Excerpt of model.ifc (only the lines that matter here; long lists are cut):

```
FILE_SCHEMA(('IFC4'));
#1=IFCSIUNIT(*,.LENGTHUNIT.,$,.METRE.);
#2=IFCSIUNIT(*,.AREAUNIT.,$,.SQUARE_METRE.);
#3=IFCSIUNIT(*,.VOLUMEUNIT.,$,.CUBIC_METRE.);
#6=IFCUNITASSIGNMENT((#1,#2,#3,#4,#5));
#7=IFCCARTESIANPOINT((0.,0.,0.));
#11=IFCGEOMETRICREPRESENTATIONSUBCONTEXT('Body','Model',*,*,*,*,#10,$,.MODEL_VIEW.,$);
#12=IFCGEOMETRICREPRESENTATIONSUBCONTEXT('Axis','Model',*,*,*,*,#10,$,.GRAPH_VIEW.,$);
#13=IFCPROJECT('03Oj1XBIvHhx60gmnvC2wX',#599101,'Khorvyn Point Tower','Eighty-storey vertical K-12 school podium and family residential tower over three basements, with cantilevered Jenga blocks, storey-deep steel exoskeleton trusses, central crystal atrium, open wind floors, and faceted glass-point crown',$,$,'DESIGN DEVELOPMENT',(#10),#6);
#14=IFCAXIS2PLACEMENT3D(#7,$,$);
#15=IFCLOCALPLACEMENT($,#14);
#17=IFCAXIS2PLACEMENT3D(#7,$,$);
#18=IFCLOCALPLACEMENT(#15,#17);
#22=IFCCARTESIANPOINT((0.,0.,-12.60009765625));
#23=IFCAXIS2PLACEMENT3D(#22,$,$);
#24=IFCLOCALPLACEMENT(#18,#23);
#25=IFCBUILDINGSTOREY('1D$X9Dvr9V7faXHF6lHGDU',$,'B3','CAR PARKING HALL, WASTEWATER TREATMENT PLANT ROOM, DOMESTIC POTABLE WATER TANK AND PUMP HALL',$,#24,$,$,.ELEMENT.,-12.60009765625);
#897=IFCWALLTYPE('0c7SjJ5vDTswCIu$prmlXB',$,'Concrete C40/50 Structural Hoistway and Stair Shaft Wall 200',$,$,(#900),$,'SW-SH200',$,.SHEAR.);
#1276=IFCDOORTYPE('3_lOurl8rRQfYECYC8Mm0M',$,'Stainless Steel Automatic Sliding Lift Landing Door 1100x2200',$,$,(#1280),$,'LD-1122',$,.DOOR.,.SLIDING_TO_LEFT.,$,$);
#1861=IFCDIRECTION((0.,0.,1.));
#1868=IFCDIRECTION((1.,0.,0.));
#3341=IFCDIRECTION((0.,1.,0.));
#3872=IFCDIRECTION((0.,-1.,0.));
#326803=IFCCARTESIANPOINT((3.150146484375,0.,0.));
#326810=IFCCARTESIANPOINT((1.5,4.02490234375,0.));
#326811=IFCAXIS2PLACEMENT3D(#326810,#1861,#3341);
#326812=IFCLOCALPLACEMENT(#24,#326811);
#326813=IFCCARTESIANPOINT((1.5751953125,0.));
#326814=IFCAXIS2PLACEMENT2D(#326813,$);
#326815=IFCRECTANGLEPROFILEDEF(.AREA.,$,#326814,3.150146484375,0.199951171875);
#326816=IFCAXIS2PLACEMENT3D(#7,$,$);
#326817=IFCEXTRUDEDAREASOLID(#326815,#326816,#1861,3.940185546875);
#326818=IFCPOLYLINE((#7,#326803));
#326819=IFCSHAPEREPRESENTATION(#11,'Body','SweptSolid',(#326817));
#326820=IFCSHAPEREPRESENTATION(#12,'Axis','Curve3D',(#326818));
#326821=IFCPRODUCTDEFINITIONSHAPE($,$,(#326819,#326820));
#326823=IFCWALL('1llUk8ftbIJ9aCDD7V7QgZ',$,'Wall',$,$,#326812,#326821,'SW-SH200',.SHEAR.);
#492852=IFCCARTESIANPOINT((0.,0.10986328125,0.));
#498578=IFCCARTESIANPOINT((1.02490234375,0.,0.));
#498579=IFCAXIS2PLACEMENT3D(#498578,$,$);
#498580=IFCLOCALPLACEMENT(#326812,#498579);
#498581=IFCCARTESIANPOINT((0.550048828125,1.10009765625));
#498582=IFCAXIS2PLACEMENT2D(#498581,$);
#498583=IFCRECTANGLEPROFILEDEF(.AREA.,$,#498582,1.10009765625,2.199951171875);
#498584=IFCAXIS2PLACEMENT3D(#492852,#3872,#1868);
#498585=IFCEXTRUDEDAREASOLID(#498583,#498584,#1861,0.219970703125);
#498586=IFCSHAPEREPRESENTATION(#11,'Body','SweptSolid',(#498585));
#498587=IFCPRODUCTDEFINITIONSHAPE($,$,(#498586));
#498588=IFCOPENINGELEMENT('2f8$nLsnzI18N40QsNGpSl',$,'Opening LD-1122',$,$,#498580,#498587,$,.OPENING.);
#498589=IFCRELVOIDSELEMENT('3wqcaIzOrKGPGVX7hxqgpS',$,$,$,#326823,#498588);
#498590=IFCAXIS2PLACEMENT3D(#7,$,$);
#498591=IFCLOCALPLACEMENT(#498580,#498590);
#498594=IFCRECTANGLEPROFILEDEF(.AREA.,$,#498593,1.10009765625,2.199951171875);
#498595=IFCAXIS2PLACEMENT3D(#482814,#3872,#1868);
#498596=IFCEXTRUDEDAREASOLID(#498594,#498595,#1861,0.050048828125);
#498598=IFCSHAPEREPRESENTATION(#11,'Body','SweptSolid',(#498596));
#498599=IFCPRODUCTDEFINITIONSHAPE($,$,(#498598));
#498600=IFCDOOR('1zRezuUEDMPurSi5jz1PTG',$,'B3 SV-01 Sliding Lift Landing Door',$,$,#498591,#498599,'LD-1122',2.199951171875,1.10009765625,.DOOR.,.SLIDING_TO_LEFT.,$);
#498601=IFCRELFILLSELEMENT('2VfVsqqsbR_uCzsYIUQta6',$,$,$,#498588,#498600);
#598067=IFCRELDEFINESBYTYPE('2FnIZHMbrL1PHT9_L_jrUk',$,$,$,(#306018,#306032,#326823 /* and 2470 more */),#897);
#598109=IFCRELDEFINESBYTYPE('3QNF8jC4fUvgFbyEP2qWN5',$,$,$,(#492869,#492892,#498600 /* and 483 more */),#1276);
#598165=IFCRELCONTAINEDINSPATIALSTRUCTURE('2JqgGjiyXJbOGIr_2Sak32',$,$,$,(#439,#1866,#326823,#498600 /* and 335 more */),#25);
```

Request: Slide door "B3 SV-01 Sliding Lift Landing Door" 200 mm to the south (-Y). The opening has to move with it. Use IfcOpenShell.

```python
import ifcopenshell
import ifcopenshell.api.geometry
import ifcopenshell.util.placement
import ifcopenshell.util.unit

model = ifcopenshell.open("model.ifc")
unit_scale = ifcopenshell.util.unit.calculate_unit_scale(model)

door = model.by_guid("1zRezuUEDMPurSi5jz1PTG")
opening = door.FillsVoids[0].RelatingOpeningElement
wall = opening.VoidsElements[0].RelatingBuildingElement

wall_matrix = ifcopenshell.util.placement.get_local_placement(wall.ObjectPlacement)
shift = wall_matrix[:3, 0] * -0.2 / unit_scale
before = ifcopenshell.util.placement.get_local_placement(door.ObjectPlacement)[:3, 3].copy()

# The door is placed relative to its opening, so it follows when the opening moves.
matrix = ifcopenshell.util.placement.get_local_placement(opening.ObjectPlacement)
matrix[:3, 3] += shift
ifcopenshell.api.geometry.edit_object_placement(
    model, product=opening, matrix=matrix, is_si=False, should_transform_children=True
)

after = ifcopenshell.util.placement.get_local_placement(door.ObjectPlacement)[:3, 3]
print("door moved by", (after - before).round(3) + 0.0)

model.write("model-out.ifc")
```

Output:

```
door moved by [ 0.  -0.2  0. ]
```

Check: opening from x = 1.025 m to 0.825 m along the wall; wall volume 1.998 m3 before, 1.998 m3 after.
